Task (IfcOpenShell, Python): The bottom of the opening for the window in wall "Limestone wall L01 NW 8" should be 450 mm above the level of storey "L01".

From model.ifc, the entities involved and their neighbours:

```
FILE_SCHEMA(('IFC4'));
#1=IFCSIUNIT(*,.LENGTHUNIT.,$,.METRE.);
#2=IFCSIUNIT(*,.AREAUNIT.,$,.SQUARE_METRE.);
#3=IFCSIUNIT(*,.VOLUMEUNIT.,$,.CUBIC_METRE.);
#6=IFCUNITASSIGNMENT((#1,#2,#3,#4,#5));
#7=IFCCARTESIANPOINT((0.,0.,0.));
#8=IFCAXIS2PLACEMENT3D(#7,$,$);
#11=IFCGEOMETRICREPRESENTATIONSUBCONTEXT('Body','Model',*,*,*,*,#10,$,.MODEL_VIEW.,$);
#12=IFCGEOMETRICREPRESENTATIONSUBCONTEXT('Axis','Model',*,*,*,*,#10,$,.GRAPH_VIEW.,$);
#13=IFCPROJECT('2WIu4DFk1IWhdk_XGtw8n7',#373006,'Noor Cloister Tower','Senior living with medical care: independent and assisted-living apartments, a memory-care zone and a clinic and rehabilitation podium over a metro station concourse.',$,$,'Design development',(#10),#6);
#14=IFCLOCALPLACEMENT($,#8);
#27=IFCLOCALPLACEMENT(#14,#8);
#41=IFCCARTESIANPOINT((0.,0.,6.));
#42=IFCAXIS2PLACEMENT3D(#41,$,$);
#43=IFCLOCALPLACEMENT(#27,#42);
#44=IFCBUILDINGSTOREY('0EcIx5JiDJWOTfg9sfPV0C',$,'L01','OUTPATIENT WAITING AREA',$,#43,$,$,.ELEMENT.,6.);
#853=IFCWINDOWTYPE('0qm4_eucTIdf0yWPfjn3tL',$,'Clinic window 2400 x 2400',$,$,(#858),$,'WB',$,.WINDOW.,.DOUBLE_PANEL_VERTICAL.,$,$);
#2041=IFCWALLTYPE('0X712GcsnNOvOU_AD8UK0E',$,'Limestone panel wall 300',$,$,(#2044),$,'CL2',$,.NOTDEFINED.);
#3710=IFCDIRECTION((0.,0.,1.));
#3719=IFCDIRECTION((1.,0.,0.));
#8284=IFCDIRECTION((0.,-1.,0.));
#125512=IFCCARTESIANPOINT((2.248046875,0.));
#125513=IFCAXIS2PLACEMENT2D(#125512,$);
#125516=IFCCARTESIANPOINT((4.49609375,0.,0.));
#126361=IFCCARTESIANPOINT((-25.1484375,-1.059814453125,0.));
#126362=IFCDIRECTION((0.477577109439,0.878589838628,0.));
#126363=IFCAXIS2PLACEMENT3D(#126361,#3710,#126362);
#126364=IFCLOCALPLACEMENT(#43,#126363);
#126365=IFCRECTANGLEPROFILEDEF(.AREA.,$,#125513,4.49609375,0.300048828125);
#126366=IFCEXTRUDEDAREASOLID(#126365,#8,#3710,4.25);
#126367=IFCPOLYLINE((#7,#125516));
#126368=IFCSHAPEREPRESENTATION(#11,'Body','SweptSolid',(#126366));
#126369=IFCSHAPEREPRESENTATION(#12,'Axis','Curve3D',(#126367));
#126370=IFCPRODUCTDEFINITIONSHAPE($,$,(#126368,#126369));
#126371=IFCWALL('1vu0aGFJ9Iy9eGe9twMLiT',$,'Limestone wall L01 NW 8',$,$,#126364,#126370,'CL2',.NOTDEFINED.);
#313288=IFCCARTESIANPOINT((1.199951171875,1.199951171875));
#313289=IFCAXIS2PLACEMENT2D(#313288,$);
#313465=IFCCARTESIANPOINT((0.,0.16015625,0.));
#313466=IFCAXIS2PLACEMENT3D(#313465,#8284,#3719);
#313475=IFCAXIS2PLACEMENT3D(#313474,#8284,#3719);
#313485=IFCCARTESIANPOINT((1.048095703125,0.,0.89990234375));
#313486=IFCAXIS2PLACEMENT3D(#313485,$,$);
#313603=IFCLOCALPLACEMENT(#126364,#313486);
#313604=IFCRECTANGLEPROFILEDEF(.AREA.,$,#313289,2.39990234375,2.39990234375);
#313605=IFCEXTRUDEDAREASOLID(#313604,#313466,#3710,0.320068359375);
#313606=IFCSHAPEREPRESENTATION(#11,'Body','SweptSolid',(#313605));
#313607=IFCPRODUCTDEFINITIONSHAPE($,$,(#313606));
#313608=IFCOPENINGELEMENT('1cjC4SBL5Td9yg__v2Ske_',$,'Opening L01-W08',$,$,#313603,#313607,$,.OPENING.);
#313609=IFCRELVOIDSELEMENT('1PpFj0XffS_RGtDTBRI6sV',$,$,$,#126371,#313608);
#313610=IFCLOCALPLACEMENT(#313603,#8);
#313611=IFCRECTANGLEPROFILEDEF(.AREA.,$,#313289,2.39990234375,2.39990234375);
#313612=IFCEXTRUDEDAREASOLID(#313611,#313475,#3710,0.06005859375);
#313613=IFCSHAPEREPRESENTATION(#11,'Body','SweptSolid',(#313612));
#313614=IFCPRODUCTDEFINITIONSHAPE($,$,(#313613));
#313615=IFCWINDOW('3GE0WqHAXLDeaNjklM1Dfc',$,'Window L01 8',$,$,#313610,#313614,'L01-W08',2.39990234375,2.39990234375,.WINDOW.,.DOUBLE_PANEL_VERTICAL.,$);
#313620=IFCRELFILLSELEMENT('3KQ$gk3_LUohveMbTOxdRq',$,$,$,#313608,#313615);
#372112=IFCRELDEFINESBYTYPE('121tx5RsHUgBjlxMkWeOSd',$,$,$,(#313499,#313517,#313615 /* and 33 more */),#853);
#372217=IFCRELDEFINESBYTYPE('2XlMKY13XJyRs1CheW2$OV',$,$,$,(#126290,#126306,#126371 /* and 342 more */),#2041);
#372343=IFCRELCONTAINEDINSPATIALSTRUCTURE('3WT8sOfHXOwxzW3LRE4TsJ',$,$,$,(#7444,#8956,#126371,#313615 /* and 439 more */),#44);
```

```python
import numpy as np
import ifcopenshell
import ifcopenshell.api.geometry
import ifcopenshell.geom
import ifcopenshell.util.element
import ifcopenshell.util.placement
import ifcopenshell.util.shape
import ifcopenshell.util.unit

model = ifcopenshell.open("model.ifc")
unit_scale = ifcopenshell.util.unit.calculate_unit_scale(model)

window = model.by_guid("3GE0WqHAXLDeaNjklM1Dfc")
opening = window.FillsVoids[0].RelatingOpeningElement
storey = ifcopenshell.util.element.get_container(window, ifc_class="IfcBuildingStorey")
level = ifcopenshell.util.placement.get_local_placement(storey.ObjectPlacement)[2, 3]

# The opening's origin need not be at the sill, so measure its lowest point.
shape = ifcopenshell.geom.create_shape(ifcopenshell.geom.settings(), opening)
bottom = ifcopenshell.util.shape.get_shape_bottom_elevation(shape, shape.geometry) / unit_scale
dz = level + 0.45 - bottom

shift = np.array([0.0, 0.0, dz])
# The window is placed relative to its opening, so it follows when the opening moves.
matrix = ifcopenshell.util.placement.get_local_placement(opening.ObjectPlacement)
matrix[:3, 3] += shift
ifcopenshell.api.geometry.edit_object_placement(
    model, product=opening, matrix=matrix, is_si=False, should_transform_children=True
)

print(f"moved by {dz * unit_scale:+.3f} m")

model.write("model_edited.ifc")
```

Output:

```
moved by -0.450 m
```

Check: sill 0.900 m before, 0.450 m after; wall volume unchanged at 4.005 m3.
